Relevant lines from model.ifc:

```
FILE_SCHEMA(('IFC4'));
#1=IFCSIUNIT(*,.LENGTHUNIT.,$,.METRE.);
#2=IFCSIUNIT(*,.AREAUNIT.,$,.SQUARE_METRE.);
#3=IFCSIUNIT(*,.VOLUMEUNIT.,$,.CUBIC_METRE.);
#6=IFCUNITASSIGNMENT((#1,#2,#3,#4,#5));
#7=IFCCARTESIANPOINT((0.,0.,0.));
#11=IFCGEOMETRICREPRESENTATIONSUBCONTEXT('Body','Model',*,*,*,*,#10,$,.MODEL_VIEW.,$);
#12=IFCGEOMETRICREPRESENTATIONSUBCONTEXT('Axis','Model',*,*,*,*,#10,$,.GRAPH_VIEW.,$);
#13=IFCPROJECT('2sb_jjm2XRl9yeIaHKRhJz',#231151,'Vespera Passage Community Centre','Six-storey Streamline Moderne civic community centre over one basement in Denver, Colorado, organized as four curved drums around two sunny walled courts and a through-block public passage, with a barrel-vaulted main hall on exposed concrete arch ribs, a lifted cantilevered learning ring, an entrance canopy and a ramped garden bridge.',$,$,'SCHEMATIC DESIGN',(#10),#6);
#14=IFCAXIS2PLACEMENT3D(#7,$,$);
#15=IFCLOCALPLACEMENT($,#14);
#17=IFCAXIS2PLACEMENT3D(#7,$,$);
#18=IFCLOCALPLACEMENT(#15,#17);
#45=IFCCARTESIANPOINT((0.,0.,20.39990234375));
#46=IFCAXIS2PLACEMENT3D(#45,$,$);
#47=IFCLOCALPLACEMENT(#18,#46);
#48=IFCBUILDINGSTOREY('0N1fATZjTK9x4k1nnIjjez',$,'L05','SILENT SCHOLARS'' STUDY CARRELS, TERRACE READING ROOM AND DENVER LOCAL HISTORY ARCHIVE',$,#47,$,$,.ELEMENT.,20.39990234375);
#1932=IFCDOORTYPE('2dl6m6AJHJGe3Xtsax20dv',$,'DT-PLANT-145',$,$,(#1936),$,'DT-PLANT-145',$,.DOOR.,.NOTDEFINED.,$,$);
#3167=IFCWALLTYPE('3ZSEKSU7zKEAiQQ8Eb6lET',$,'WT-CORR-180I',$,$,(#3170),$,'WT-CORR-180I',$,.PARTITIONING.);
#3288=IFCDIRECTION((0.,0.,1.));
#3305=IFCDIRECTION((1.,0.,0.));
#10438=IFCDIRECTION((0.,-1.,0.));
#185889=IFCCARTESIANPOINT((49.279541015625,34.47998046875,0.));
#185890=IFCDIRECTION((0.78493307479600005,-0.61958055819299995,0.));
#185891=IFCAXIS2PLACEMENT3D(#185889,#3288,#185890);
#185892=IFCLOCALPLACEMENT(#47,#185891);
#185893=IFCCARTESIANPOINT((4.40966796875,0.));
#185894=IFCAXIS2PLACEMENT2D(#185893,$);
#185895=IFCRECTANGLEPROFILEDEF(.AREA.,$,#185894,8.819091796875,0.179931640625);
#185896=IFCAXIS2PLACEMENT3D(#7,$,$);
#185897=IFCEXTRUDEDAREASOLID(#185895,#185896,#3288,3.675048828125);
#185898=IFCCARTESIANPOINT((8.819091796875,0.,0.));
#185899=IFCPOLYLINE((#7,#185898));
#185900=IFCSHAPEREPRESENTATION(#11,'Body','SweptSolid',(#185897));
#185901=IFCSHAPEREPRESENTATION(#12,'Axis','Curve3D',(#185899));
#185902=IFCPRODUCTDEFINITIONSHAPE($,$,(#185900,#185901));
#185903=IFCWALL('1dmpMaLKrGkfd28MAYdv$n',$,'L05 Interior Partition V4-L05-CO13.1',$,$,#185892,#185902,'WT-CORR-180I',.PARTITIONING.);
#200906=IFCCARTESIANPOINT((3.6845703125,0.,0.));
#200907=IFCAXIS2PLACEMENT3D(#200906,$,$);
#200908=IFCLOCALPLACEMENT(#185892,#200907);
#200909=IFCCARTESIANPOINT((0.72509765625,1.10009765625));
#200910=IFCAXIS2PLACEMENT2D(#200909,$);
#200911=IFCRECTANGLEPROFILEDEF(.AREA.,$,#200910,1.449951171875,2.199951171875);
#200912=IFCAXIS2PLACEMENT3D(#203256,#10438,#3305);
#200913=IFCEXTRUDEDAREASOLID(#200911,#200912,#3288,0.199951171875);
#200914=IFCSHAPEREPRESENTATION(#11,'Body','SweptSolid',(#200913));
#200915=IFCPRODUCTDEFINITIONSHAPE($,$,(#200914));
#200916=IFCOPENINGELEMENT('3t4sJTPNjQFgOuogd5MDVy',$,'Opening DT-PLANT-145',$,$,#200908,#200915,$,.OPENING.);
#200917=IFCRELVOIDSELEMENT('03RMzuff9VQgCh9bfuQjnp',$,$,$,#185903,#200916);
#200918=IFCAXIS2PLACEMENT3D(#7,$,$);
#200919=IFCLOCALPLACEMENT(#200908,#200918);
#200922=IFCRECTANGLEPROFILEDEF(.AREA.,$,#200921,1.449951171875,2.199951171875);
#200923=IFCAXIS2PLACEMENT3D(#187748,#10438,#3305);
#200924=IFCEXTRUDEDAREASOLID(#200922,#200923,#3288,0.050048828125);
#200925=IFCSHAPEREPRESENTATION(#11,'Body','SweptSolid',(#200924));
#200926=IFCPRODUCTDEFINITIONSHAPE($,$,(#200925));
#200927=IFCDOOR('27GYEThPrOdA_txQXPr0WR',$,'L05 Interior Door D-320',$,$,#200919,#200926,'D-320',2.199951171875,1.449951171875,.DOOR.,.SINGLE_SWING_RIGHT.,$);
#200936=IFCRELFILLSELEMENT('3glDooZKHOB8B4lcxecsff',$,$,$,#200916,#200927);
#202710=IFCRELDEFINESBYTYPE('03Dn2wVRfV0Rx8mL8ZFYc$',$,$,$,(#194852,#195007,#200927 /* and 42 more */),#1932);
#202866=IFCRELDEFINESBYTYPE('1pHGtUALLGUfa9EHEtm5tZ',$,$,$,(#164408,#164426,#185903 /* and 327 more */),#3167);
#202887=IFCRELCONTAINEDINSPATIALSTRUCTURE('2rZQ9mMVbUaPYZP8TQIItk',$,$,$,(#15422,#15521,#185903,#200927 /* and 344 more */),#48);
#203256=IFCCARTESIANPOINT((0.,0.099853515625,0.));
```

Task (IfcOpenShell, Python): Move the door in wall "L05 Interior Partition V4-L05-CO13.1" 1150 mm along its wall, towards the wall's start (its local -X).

```python
import ifcopenshell
import ifcopenshell.api.geometry
import ifcopenshell.util.placement

model = ifcopenshell.open("model.ifc")

door = model.by_guid("27GYEThPrOdA_txQXPr0WR")
opening = door.FillsVoids[0].RelatingOpeningElement
wall = opening.VoidsElements[0].RelatingBuildingElement

wall_matrix = ifcopenshell.util.placement.get_local_placement(wall.ObjectPlacement)
shift = wall_matrix[:3, 0] * -1.15
before = ifcopenshell.util.placement.get_local_placement(door.ObjectPlacement)[:3, 3].copy()

# The door is placed relative to its opening, so it follows when the opening moves.
matrix = ifcopenshell.util.placement.get_local_placement(opening.ObjectPlacement)
matrix[:3, 3] += shift
ifcopenshell.api.geometry.edit_object_placement(
    model, product=opening, matrix=matrix, is_si=False, should_transform_children=True
)

after = ifcopenshell.util.placement.get_local_placement(door.ObjectPlacement)[:3, 3]
print("door moved by", (after - before).round(3) + 0.0)

model.write("model_v2.ifc")
```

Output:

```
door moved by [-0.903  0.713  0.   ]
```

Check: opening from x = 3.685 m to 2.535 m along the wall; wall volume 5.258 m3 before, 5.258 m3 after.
